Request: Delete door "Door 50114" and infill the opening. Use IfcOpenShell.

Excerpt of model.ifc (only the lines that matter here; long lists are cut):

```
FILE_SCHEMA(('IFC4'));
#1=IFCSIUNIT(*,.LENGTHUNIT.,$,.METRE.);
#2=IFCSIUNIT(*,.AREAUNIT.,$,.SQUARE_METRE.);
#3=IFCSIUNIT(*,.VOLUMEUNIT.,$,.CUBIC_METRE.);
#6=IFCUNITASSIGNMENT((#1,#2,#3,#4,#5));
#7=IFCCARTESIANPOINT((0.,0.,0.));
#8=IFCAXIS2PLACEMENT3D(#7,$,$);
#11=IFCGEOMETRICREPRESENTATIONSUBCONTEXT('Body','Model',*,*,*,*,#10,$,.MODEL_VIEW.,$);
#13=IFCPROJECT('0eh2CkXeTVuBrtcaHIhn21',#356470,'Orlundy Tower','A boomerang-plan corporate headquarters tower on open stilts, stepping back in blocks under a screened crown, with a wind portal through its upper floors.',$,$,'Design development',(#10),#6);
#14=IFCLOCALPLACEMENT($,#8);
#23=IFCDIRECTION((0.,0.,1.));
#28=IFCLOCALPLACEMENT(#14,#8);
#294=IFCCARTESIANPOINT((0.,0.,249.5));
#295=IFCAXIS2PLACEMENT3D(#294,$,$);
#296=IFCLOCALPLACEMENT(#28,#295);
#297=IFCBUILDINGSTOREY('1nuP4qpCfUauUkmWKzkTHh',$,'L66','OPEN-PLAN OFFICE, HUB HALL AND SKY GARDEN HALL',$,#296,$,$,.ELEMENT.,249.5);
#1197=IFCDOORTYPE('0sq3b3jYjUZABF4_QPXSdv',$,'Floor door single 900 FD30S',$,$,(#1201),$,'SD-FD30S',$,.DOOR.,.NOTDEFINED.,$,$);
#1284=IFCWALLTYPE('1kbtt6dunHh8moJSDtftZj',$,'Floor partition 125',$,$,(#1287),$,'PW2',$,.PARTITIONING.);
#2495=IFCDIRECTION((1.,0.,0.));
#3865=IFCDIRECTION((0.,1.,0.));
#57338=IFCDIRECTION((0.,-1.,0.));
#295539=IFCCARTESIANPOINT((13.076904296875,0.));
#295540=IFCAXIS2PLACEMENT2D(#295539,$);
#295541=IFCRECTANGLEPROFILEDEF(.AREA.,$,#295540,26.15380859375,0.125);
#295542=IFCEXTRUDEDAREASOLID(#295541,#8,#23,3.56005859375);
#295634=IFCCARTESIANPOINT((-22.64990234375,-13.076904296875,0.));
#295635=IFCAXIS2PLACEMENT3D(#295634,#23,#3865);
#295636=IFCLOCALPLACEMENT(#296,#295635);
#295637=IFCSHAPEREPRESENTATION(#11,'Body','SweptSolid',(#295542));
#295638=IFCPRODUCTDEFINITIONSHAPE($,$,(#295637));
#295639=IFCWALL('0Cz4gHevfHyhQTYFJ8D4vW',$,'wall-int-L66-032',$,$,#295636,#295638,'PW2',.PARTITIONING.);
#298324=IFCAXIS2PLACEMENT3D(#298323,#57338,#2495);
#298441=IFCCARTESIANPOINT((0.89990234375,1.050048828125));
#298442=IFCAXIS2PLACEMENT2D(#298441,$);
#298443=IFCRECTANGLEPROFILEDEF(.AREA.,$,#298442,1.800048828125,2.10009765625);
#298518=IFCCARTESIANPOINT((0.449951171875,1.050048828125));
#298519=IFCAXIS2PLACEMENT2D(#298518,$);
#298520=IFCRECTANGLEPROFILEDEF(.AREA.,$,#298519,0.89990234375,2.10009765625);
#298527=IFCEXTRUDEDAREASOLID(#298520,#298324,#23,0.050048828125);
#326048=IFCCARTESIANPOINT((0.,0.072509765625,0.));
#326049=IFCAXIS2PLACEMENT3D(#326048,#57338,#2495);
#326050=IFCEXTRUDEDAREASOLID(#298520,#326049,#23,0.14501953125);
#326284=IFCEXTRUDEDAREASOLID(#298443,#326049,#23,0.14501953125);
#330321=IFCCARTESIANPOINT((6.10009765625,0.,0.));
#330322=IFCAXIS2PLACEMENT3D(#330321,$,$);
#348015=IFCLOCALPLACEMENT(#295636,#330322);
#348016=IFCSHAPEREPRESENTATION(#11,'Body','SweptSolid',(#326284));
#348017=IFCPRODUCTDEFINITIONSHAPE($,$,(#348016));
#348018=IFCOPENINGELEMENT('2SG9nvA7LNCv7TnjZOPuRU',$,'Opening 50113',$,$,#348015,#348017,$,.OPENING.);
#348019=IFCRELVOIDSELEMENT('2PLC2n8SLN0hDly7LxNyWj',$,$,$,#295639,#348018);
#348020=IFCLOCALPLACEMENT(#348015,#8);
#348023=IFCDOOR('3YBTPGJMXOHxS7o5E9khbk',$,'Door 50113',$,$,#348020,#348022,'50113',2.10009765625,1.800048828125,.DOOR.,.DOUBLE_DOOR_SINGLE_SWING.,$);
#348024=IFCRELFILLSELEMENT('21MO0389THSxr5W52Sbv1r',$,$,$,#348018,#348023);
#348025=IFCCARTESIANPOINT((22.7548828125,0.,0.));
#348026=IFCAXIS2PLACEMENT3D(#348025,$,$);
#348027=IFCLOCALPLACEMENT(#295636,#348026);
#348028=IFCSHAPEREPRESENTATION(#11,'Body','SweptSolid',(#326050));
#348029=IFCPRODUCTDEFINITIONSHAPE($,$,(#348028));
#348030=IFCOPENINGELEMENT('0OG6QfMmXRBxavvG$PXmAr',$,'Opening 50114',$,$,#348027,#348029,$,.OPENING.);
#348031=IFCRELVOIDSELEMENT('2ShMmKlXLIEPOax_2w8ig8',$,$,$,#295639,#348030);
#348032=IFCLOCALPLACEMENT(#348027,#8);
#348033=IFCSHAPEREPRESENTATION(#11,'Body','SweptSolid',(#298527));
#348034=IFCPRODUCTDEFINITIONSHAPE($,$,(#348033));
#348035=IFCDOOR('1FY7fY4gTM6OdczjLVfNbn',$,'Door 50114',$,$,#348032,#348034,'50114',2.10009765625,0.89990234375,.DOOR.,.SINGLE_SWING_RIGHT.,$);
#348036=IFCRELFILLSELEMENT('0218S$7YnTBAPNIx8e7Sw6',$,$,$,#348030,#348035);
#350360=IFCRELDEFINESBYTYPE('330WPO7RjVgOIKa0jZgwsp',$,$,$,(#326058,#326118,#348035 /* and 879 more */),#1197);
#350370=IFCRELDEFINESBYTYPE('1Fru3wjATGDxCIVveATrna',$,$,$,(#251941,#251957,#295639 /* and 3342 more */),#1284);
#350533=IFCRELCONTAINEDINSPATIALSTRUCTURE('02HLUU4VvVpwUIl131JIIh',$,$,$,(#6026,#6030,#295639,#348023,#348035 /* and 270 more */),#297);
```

```python
import ifcopenshell
import ifcopenshell.api.feature
import ifcopenshell.api.root
import ifcopenshell.geom
import ifcopenshell.util.shape

model = ifcopenshell.open("model.ifc")
settings = ifcopenshell.geom.settings()


def volume(element):
    """Net volume in cubic metres, openings subtracted."""
    shape = ifcopenshell.geom.create_shape(settings, element)
    return ifcopenshell.util.shape.get_volume(shape.geometry)


door = model.by_id(348035)
opening = door.FillsVoids[0].RelatingOpeningElement
wall = opening.VoidsElements[0].RelatingBuildingElement
before = volume(wall)

ifcopenshell.api.root.remove_product(model, product=door)
ifcopenshell.api.feature.remove_feature(model, feature=opening)

after = volume(wall)

print(f"wall volume {before:.3f} -> {after:.3f} m3")

model.write("model-out.ifc")
```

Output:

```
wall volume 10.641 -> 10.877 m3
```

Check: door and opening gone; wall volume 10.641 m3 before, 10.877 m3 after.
